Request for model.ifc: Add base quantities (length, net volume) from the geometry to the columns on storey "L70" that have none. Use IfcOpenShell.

First a look at what the model holds.

```python
import ifcopenshell
import ifcopenshell.util.element
import ifcopenshell.util.unit

model = ifcopenshell.open("model.ifc")
print(model.schema)
for unit_type in ("LENGTHUNIT", "AREAUNIT", "VOLUMEUNIT"):
    print(unit_type, ifcopenshell.util.unit.calculate_unit_scale(model, unit_type))
storey = next(s for s in model.by_type("IfcBuildingStorey") if s.Name == "L70")
columns = [e for e in ifcopenshell.util.element.get_decomposition(storey) if e.is_a("IfcColumn")]
for e in sorted(columns, key=lambda e: e.id()):
    print(e.id(), e.is_a(), e.Name, list(ifcopenshell.util.element.get_psets(e, qtos_only=True)), sep=" | ")
```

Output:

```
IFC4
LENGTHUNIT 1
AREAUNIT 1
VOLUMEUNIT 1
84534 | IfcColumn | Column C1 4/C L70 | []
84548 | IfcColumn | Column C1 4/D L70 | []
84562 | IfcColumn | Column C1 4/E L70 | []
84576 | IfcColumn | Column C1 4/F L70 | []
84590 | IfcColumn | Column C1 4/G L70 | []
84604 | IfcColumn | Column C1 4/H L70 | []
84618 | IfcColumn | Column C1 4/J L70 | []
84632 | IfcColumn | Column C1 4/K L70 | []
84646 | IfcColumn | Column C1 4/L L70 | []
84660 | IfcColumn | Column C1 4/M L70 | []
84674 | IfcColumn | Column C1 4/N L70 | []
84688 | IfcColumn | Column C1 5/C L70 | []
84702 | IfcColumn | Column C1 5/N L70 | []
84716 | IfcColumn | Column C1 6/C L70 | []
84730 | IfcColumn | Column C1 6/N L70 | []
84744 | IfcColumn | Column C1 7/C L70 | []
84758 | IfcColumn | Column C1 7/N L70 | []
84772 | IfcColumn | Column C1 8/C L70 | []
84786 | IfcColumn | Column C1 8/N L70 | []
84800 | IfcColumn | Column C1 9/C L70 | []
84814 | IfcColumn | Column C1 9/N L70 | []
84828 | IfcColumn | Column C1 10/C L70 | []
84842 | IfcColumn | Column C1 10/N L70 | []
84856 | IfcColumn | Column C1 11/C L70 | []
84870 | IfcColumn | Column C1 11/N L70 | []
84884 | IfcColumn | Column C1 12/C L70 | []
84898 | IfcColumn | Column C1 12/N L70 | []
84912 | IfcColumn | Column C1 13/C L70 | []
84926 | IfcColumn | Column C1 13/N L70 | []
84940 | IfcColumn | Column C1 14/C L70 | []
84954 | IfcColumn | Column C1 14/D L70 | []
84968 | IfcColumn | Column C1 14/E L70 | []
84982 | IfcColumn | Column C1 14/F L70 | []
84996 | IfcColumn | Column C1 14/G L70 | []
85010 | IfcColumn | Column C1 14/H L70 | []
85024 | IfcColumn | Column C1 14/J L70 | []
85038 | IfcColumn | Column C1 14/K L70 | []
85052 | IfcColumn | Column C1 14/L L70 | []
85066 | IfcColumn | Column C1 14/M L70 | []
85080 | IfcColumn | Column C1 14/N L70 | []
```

```python
import ifcopenshell
import ifcopenshell.api.pset
import ifcopenshell.geom
import ifcopenshell.util.element
import ifcopenshell.util.shape
import ifcopenshell.util.unit

model = ifcopenshell.open("model.ifc")
unit_scale = ifcopenshell.util.unit.calculate_unit_scale(model)
volume_scale = ifcopenshell.util.unit.calculate_unit_scale(model, "VOLUMEUNIT")
settings = ifcopenshell.geom.settings()

storey = next(s for s in model.by_type("IfcBuildingStorey") if s.Name == "L70")
columns = [e for e in ifcopenshell.util.element.get_decomposition(storey) if e.is_a("IfcColumn")]

for e in sorted(columns, key=lambda e: e.id()):
    if ifcopenshell.util.element.get_psets(e, qtos_only=True, should_inherit=False):
        continue
    # Geometry comes back in metres, in the element's own axes.
    shape = ifcopenshell.geom.create_shape(settings, e)
    values = {
        "Length": ifcopenshell.util.shape.get_z(shape.geometry) / unit_scale,
        "NetVolume": ifcopenshell.util.shape.get_volume(shape.geometry) / volume_scale,
    }
    qto = ifcopenshell.api.pset.add_qto(model, product=e, name="Qto_ColumnBaseQuantities")
    ifcopenshell.api.pset.edit_qto(model, qto=qto, properties=values)
    print(e.id(), {k: round(v, 3) for k, v in values.items()})

model.write("model_updated.ifc")
```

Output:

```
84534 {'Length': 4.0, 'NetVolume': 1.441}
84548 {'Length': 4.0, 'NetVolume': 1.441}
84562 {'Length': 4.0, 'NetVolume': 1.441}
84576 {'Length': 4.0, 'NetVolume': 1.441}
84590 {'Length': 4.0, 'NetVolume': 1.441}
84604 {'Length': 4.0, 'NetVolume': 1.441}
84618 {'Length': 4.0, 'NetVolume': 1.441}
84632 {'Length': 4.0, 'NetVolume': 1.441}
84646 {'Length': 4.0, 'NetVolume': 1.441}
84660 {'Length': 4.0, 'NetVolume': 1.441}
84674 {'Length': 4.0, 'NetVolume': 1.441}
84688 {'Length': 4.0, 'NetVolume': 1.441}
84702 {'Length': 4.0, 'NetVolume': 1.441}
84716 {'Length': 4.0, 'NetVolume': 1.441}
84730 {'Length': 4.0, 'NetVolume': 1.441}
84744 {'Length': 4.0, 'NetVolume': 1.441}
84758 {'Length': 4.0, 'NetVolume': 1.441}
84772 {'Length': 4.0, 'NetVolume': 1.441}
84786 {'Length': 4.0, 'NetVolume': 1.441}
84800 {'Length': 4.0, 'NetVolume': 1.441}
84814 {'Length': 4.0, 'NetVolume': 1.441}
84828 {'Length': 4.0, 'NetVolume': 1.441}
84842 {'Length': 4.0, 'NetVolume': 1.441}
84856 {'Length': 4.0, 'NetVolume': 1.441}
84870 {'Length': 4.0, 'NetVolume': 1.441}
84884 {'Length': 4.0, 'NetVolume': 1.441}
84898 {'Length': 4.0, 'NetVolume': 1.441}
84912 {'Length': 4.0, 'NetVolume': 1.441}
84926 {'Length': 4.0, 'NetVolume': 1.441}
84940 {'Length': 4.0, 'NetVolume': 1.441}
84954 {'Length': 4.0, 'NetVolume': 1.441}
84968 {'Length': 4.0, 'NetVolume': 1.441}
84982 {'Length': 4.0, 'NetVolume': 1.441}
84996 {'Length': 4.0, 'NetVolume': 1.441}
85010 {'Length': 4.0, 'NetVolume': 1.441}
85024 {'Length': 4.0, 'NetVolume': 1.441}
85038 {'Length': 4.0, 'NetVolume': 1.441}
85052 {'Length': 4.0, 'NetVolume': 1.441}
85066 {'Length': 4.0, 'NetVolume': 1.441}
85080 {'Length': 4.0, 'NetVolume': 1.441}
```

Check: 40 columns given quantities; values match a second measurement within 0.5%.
